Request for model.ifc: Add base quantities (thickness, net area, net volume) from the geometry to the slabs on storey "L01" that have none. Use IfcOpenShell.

First a look at what the model holds.

```python
import ifcopenshell
import ifcopenshell.util.element
import ifcopenshell.util.unit

model = ifcopenshell.open("model.ifc")
print(model.schema)
for unit_type in ("LENGTHUNIT", "AREAUNIT", "VOLUMEUNIT"):
    print(unit_type, ifcopenshell.util.unit.calculate_unit_scale(model, unit_type))
storey = next(s for s in model.by_type("IfcBuildingStorey") if s.Name == "L01")
slabs = [e for e in ifcopenshell.util.element.get_decomposition(storey) if e.is_a("IfcSlab")]
for e in sorted(slabs, key=lambda e: e.id()):
    print(e.id(), e.is_a(), e.Name, list(ifcopenshell.util.element.get_psets(e, qtos_only=True)), sep=" | ")
```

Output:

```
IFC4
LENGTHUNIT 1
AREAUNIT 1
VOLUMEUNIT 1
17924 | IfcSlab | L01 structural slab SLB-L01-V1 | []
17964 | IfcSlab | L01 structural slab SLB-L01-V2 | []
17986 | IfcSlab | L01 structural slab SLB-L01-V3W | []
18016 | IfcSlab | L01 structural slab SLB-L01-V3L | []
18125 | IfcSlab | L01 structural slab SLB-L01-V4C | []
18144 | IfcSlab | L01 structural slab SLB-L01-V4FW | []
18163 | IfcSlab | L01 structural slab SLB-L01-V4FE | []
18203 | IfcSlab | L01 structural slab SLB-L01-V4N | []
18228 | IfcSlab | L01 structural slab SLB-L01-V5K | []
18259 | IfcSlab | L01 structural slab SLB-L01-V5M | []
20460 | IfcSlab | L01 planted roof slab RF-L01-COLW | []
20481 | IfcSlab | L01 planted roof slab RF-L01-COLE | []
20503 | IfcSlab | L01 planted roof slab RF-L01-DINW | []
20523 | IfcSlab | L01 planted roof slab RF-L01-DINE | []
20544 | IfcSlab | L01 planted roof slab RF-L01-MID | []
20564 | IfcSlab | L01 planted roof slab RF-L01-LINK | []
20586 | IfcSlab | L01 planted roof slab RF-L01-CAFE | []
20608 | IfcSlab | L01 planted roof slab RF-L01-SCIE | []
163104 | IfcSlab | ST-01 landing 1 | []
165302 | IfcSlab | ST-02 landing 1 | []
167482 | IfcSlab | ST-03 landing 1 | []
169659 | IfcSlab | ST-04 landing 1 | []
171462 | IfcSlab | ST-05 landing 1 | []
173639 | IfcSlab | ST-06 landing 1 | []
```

```python
import ifcopenshell
import ifcopenshell.api.pset
import ifcopenshell.geom
import ifcopenshell.util.element
import ifcopenshell.util.shape
import ifcopenshell.util.unit

model = ifcopenshell.open("model.ifc")
unit_scale = ifcopenshell.util.unit.calculate_unit_scale(model)
area_scale = ifcopenshell.util.unit.calculate_unit_scale(model, "AREAUNIT")
volume_scale = ifcopenshell.util.unit.calculate_unit_scale(model, "VOLUMEUNIT")
settings = ifcopenshell.geom.settings()

storey = next(s for s in model.by_type("IfcBuildingStorey") if s.Name == "L01")
slabs = [e for e in ifcopenshell.util.element.get_decomposition(storey) if e.is_a("IfcSlab")]

for e in sorted(slabs, key=lambda e: e.id()):
    if ifcopenshell.util.element.get_psets(e, qtos_only=True, should_inherit=False):
        continue
    # Geometry comes back in metres, in the element's own axes.
    shape = ifcopenshell.geom.create_shape(settings, e)
    values = {
        "Width": ifcopenshell.util.shape.get_z(shape.geometry) / unit_scale,
        "NetArea": ifcopenshell.util.shape.get_footprint_area(shape.geometry) / area_scale,
        "NetVolume": ifcopenshell.util.shape.get_volume(shape.geometry) / volume_scale,
    }
    qto = ifcopenshell.api.pset.add_qto(model, product=e, name="Qto_SlabBaseQuantities")
    ifcopenshell.api.pset.edit_qto(model, qto=qto, properties=values)
    print(e.id(), {k: round(v, 3) for k, v in values.items()})

model.write("model_edited.ifc")
```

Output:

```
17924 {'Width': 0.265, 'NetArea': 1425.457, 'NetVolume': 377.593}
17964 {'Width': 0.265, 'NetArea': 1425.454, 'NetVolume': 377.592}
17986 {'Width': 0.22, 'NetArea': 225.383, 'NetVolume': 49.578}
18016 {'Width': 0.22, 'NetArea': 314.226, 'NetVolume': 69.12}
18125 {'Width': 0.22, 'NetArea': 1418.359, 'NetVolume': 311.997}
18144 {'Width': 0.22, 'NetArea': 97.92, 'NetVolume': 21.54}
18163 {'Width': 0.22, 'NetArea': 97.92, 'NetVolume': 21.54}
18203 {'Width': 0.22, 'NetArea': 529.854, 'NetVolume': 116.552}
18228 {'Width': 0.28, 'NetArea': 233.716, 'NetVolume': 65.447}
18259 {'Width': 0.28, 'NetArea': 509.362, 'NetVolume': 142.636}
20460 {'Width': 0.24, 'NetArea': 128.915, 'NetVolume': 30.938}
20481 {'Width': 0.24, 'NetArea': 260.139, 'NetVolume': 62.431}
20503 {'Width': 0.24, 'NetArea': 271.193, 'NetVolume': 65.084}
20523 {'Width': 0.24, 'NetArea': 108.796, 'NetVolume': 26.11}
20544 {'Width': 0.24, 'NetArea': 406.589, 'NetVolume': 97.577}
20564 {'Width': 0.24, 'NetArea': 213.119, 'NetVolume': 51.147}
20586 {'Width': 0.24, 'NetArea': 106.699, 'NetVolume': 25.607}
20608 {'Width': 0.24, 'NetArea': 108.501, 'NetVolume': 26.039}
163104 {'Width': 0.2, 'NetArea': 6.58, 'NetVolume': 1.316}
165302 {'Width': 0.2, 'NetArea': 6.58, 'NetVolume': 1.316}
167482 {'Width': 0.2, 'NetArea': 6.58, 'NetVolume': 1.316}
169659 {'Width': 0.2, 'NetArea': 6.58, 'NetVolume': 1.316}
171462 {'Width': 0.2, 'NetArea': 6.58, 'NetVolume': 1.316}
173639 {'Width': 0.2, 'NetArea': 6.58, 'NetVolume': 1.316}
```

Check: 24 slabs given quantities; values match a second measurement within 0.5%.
